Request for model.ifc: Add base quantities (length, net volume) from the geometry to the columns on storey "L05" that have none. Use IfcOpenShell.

First a look at what the model holds.

```python
import ifcopenshell
import ifcopenshell.util.element
import ifcopenshell.util.unit

model = ifcopenshell.open("model.ifc")
print(model.schema)
for unit_type in ("LENGTHUNIT", "AREAUNIT", "VOLUMEUNIT"):
    print(unit_type, ifcopenshell.util.unit.calculate_unit_scale(model, unit_type))
storey = next(s for s in model.by_type("IfcBuildingStorey") if s.Name == "L05")
columns = [e for e in ifcopenshell.util.element.get_decomposition(storey) if e.is_a("IfcColumn")]
for e in sorted(columns, key=lambda e: e.id()):
    print(e.id(), e.is_a(), e.Name, list(ifcopenshell.util.element.get_psets(e, qtos_only=True)), sep=" | ")
```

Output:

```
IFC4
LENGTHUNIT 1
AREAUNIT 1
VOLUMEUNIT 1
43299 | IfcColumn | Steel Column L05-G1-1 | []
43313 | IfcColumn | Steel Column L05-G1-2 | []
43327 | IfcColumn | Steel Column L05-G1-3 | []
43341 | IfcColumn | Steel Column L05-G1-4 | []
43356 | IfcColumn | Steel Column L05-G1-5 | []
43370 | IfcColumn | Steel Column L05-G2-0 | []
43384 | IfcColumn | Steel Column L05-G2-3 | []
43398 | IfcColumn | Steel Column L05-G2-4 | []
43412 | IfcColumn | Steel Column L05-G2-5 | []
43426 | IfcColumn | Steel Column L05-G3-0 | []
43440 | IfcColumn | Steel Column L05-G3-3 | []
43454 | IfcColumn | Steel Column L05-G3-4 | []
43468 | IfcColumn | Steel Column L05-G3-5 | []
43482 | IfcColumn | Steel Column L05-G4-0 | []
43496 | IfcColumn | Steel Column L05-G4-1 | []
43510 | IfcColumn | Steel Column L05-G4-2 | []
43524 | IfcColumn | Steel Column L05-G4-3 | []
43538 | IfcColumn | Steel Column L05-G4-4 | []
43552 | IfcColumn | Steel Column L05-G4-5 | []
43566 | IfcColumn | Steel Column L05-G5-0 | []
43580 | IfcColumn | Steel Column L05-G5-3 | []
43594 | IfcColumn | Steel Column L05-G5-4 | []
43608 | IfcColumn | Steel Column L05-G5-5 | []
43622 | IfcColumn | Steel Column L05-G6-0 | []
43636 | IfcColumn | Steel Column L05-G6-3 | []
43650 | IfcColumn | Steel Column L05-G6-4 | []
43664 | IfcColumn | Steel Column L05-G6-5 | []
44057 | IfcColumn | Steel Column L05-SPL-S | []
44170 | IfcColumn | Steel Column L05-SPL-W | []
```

```python
import ifcopenshell
import ifcopenshell.api.pset
import ifcopenshell.geom
import ifcopenshell.util.element
import ifcopenshell.util.shape
import ifcopenshell.util.unit

model = ifcopenshell.open("model.ifc")
unit_scale = ifcopenshell.util.unit.calculate_unit_scale(model)
volume_scale = ifcopenshell.util.unit.calculate_unit_scale(model, "VOLUMEUNIT")
settings = ifcopenshell.geom.settings()

storey = next(s for s in model.by_type("IfcBuildingStorey") if s.Name == "L05")
columns = [e for e in ifcopenshell.util.element.get_decomposition(storey) if e.is_a("IfcColumn")]

for e in sorted(columns, key=lambda e: e.id()):
    if ifcopenshell.util.element.get_psets(e, qtos_only=True, should_inherit=False):
        continue
    # Geometry comes back in metres, in the element's own axes.
    shape = ifcopenshell.geom.create_shape(settings, e)
    values = {
        "Length": ifcopenshell.util.shape.get_z(shape.geometry) / unit_scale,
        "NetVolume": ifcopenshell.util.shape.get_volume(shape.geometry) / volume_scale,
    }
    qto = ifcopenshell.api.pset.add_qto(model, product=e, name="Qto_ColumnBaseQuantities")
    ifcopenshell.api.pset.edit_qto(model, qto=qto, properties=values)
    print(e.id(), {k: round(v, 3) for k, v in values.items()})

model.write("model-out.ifc")
```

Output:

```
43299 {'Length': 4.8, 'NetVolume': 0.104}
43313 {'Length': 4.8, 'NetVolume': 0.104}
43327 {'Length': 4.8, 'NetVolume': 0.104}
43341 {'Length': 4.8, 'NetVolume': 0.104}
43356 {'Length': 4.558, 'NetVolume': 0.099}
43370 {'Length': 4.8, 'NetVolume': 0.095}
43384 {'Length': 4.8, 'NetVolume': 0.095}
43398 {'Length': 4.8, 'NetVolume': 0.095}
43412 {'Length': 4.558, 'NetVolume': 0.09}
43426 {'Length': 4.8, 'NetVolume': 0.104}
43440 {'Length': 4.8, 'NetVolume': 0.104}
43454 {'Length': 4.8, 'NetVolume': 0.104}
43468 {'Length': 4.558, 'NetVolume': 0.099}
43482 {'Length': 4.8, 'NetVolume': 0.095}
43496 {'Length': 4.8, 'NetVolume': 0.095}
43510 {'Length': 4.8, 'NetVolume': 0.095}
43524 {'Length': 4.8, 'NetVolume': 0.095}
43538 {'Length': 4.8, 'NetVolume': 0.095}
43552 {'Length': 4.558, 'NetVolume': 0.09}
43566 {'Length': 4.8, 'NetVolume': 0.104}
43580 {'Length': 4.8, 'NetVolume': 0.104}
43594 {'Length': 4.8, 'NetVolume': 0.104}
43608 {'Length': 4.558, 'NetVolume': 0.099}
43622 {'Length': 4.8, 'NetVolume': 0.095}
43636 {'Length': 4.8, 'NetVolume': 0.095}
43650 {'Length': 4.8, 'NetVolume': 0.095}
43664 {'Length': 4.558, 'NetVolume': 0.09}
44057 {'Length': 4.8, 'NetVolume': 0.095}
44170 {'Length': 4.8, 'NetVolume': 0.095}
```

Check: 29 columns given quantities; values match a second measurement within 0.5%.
